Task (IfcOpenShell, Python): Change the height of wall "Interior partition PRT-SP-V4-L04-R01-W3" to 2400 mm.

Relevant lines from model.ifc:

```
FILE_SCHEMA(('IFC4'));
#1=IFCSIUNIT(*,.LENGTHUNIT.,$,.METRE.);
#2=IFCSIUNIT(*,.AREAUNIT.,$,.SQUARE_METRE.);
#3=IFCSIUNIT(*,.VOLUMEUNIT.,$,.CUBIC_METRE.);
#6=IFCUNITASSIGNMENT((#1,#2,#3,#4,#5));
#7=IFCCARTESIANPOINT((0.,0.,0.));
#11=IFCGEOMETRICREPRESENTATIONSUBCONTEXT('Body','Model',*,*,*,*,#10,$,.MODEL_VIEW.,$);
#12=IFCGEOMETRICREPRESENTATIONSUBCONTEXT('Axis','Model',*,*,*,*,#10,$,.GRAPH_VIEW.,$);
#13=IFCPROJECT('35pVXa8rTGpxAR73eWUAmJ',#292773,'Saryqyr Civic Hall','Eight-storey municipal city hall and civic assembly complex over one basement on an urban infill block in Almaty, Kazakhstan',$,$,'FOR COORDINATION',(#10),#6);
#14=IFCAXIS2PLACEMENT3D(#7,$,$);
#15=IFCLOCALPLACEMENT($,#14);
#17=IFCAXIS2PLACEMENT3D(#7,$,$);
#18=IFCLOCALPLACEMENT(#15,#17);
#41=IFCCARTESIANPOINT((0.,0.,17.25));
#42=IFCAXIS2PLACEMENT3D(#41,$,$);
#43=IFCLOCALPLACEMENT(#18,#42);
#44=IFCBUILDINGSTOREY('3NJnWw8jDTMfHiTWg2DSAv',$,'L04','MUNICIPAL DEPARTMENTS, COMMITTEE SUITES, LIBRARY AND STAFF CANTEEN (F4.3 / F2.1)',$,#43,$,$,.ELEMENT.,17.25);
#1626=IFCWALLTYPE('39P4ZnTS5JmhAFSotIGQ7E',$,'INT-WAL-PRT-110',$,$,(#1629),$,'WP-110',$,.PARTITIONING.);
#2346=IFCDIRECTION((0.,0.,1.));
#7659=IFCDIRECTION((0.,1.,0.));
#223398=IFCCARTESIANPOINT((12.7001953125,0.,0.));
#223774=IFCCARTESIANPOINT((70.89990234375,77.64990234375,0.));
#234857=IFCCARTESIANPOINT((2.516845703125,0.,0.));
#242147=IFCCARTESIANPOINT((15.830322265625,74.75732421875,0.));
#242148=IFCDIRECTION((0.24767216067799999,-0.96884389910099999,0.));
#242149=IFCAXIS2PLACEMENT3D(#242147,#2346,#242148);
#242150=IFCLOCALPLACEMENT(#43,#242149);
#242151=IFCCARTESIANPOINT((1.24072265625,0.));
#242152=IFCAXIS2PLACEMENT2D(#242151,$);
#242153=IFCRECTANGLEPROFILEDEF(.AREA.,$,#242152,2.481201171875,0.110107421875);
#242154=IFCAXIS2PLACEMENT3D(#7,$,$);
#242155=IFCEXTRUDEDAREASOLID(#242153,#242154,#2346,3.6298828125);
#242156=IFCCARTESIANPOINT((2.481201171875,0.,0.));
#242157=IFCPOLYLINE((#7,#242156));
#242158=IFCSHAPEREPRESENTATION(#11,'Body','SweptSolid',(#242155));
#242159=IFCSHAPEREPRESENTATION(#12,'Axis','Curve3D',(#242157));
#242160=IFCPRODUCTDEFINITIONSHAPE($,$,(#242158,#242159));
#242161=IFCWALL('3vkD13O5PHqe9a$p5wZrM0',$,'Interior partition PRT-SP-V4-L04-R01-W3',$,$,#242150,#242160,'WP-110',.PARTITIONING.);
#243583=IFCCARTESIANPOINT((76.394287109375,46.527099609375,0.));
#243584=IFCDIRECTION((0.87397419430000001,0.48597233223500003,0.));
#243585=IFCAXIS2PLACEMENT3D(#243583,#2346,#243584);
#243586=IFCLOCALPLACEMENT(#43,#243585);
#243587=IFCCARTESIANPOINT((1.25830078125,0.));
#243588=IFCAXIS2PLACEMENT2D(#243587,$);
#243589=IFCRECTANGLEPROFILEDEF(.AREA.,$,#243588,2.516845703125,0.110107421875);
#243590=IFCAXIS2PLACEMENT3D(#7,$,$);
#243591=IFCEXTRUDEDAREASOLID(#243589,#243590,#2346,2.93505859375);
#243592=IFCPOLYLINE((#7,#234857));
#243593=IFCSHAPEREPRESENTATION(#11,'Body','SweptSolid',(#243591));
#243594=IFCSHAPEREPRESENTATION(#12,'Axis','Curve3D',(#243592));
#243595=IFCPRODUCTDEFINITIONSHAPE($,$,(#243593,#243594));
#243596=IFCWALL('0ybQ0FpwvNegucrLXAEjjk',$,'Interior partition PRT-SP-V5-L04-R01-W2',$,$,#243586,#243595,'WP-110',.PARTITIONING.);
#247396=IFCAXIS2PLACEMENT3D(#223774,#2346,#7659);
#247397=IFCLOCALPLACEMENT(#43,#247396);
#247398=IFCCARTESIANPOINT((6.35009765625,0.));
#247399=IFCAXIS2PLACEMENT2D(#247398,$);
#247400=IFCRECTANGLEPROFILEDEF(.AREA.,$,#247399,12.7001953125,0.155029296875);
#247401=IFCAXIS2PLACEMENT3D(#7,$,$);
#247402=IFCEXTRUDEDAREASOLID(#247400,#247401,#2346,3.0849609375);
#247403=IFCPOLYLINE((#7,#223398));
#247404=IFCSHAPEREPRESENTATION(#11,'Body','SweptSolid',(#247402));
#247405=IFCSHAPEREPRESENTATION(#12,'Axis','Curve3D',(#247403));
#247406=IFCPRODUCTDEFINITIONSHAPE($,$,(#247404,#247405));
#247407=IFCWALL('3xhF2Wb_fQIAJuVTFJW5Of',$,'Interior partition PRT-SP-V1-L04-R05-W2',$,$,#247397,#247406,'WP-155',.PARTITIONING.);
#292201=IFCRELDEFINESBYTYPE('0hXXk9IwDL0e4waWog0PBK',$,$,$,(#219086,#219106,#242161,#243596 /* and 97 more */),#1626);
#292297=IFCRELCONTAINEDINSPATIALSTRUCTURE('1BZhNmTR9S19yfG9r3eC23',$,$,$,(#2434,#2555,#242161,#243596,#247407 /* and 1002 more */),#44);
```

```python
import ifcopenshell
import ifcopenshell.geom
import ifcopenshell.util.representation
import ifcopenshell.util.shape

model = ifcopenshell.open("model.ifc")
settings = ifcopenshell.geom.settings()


def volume(element):
    """Net volume in cubic metres, openings subtracted."""
    shape = ifcopenshell.geom.create_shape(settings, element)
    return ifcopenshell.util.shape.get_volume(shape.geometry)


wall = model.by_id(242161)
before = volume(wall)

body = ifcopenshell.util.representation.get_representation(wall, "Model", "Body")
solid = body.Items[0]
old_height = solid.Depth
solid.Depth = 2.4
after = volume(wall)

print(f"height {old_height:g} -> {solid.Depth:g}, volume {before:.3f} -> {after:.3f} m3")

model.write("model_rev.ifc")
```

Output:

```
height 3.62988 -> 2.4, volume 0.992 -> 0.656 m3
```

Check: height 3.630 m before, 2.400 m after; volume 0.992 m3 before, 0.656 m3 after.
